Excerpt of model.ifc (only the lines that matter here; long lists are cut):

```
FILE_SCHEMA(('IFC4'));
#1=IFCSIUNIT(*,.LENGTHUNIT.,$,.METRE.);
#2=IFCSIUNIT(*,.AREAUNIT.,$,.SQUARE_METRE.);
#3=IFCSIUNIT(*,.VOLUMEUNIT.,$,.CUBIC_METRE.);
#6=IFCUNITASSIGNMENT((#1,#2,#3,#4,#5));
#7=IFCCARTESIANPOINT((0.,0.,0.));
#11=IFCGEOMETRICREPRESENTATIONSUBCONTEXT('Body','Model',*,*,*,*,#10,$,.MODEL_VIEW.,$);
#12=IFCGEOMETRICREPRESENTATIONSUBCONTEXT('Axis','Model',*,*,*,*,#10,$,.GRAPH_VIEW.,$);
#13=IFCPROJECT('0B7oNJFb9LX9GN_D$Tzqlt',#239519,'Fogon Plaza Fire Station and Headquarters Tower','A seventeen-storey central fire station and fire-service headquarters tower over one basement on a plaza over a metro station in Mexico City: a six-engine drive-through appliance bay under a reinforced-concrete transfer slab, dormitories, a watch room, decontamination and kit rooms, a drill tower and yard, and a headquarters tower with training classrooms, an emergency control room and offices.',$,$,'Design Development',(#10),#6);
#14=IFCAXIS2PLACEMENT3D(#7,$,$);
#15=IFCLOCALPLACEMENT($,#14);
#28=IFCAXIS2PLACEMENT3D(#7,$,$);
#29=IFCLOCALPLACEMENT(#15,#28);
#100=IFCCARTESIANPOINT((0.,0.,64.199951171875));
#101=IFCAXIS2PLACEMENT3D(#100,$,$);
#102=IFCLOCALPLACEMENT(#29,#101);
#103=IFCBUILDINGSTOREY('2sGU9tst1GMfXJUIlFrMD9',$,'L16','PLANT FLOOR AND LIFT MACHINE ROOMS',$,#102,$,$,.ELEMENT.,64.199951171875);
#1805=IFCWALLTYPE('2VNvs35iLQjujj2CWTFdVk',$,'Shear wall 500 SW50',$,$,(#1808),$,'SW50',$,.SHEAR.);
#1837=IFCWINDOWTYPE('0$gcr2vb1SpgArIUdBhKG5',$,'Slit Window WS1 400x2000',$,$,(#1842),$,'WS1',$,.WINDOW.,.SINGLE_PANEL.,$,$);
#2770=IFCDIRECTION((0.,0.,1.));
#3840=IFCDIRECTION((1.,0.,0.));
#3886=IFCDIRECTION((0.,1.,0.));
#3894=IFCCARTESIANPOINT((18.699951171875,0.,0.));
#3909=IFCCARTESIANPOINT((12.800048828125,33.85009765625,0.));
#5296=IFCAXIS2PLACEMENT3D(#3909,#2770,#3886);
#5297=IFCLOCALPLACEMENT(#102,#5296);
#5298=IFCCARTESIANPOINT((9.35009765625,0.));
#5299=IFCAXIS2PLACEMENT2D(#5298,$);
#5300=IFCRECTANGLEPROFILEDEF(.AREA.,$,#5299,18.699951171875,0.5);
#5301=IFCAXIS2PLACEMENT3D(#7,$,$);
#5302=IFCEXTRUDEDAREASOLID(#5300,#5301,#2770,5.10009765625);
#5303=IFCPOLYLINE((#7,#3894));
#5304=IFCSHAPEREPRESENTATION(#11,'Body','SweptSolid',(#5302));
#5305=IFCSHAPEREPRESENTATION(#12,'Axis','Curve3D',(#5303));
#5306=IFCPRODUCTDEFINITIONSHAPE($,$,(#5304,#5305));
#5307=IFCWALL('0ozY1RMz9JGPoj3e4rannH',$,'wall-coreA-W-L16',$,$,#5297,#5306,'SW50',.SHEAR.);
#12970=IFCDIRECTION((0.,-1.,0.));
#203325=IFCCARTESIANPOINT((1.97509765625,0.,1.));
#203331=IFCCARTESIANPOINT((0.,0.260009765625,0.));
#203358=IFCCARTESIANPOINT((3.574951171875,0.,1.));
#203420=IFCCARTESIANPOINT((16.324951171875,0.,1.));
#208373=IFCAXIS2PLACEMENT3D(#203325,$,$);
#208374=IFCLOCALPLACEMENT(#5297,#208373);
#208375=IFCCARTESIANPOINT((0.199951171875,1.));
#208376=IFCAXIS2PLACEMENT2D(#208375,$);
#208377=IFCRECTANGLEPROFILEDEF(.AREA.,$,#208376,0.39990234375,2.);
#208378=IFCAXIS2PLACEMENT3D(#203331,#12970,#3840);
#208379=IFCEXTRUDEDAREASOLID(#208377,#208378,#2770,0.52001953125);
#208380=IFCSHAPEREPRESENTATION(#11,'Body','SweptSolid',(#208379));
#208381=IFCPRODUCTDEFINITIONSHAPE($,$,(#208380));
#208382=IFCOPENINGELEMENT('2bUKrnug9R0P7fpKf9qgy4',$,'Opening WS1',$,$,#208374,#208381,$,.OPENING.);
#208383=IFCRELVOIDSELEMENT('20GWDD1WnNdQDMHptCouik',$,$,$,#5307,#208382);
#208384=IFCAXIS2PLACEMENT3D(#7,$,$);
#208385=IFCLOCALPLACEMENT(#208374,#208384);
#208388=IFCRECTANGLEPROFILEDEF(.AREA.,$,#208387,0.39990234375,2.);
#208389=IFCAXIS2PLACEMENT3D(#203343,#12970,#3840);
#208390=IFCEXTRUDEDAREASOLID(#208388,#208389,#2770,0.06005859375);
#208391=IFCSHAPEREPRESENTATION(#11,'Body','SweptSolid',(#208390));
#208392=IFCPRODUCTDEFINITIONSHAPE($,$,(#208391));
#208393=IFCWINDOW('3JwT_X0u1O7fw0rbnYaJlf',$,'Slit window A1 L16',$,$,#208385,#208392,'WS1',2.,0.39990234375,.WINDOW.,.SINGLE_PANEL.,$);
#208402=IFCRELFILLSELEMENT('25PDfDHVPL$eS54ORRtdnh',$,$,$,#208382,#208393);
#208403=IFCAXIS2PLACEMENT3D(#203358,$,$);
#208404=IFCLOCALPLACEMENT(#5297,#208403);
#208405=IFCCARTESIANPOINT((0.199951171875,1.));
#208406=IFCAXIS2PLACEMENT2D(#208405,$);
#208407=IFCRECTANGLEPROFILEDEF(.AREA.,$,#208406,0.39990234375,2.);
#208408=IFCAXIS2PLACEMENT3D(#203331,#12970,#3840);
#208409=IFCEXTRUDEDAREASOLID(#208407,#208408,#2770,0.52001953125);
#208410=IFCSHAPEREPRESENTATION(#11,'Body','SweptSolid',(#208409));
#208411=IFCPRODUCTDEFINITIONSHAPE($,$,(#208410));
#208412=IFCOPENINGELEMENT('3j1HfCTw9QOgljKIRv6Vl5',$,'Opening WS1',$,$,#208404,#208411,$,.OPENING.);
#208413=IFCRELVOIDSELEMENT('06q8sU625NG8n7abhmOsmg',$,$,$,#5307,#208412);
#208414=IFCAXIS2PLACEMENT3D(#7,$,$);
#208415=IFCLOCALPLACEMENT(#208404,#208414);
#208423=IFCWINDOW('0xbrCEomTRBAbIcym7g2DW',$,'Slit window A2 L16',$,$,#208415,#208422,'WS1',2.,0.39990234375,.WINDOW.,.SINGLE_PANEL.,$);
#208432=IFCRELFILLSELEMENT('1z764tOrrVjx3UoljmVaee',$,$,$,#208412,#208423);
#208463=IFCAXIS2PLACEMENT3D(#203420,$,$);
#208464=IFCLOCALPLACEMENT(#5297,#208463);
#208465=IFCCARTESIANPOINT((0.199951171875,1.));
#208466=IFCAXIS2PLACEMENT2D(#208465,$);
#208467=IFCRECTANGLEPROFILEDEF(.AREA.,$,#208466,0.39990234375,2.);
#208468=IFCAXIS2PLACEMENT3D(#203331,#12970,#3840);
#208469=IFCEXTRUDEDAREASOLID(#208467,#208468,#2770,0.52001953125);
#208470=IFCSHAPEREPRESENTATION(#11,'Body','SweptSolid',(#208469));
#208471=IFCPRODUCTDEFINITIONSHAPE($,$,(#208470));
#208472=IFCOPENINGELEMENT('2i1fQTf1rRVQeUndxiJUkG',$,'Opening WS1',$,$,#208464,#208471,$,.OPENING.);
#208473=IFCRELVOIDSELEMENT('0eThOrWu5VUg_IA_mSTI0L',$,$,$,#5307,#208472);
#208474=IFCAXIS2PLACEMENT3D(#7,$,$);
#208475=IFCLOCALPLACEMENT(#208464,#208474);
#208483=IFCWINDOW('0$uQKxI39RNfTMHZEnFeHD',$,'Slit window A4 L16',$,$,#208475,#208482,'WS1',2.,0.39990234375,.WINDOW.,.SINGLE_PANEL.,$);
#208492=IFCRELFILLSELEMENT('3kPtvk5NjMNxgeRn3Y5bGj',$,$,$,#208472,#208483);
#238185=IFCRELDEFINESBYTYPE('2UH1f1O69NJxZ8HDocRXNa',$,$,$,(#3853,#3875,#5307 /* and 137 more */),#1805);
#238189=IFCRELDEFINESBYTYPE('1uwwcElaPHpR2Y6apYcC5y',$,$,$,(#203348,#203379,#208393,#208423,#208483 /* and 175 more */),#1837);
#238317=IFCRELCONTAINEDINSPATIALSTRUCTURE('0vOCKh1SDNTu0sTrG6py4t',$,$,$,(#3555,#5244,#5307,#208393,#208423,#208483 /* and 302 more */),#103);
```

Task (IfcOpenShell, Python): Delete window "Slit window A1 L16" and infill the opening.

```python
import ifcopenshell
import ifcopenshell.api.feature
import ifcopenshell.api.root
import ifcopenshell.geom
import ifcopenshell.util.shape

model = ifcopenshell.open("model.ifc")
settings = ifcopenshell.geom.settings()


def volume(element):
    """Net volume in cubic metres, openings subtracted."""
    shape = ifcopenshell.geom.create_shape(settings, element)
    return ifcopenshell.util.shape.get_volume(shape.geometry)


window = model.by_guid("3JwT_X0u1O7fw0rbnYaJlf")
opening = window.FillsVoids[0].RelatingOpeningElement
wall = opening.VoidsElements[0].RelatingBuildingElement
before = volume(wall)

ifcopenshell.api.root.remove_product(model, product=window)
ifcopenshell.api.feature.remove_feature(model, feature=opening)

after = volume(wall)

print(f"wall volume {before:.3f} -> {after:.3f} m3")

model.write("model-out.ifc")
```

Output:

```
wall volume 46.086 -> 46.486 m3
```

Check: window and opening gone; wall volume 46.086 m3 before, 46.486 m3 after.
